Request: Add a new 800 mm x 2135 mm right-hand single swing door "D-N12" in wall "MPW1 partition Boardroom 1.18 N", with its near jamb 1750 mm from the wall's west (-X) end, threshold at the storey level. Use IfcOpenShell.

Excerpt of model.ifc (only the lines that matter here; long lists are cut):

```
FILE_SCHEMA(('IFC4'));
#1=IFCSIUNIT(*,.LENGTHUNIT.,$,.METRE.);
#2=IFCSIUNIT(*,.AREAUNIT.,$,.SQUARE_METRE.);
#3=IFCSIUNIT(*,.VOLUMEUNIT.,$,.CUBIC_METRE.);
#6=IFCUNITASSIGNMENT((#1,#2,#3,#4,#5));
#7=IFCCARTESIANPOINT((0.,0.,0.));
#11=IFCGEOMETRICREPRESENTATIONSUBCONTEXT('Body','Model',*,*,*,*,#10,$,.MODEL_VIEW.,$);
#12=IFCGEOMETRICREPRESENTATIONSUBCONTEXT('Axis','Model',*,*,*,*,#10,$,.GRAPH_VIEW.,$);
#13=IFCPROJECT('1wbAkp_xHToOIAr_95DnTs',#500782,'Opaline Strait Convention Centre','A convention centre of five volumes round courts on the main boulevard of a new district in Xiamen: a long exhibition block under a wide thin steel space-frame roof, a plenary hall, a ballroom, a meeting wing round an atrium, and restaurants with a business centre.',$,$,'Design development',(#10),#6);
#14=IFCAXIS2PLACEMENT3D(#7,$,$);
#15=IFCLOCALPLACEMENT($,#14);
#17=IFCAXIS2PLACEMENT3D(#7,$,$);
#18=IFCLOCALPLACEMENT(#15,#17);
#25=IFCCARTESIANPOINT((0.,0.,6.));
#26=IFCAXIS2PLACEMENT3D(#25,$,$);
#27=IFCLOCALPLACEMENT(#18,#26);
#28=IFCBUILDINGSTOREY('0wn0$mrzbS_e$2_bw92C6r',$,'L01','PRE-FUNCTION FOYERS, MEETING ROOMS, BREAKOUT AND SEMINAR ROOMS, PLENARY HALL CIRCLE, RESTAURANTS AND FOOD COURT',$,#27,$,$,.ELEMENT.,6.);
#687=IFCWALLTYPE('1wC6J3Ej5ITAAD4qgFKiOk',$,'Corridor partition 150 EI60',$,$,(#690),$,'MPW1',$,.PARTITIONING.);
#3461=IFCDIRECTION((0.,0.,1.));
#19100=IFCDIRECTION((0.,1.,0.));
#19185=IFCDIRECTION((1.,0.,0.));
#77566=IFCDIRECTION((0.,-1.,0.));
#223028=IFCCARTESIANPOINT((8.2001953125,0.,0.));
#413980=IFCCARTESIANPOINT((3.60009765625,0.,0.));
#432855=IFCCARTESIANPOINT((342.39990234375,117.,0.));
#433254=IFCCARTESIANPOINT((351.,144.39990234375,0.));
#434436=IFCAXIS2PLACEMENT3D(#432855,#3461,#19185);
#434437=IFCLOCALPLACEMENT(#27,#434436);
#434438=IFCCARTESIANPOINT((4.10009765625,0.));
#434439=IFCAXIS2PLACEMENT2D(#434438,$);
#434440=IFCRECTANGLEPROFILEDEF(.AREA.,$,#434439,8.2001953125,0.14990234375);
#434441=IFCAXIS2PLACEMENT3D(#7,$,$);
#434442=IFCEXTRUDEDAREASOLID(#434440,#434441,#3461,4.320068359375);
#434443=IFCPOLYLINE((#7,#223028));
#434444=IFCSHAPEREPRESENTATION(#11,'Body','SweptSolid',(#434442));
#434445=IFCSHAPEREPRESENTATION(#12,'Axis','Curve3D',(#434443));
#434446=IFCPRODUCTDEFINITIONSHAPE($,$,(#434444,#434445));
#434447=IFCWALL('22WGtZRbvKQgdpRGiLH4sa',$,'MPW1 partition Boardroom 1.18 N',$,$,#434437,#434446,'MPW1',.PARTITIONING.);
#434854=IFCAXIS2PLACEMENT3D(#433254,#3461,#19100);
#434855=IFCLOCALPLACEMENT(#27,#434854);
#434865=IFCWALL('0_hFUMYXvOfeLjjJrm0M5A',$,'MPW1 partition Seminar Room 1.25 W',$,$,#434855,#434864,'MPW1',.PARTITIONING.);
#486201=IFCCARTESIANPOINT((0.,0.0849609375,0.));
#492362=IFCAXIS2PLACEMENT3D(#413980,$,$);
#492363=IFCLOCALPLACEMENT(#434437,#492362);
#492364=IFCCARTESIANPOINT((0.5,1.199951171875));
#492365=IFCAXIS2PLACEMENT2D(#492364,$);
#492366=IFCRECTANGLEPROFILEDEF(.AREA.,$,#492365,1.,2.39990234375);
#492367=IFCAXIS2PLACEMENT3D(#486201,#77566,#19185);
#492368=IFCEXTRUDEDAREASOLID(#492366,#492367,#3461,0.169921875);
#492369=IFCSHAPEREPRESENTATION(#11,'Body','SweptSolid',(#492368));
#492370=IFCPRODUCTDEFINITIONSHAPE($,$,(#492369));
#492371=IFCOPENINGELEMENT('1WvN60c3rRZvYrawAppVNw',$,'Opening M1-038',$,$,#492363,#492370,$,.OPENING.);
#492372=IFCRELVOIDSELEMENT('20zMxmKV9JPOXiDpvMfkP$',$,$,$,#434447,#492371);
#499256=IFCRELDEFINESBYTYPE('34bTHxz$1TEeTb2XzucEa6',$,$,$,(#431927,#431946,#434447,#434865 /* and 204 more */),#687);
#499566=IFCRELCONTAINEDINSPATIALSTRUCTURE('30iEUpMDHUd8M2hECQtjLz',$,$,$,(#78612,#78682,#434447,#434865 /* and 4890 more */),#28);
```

```python
import numpy as np
import ifcopenshell
import ifcopenshell.api.feature
import ifcopenshell.api.geometry
import ifcopenshell.api.root
import ifcopenshell.api.spatial
import ifcopenshell.geom
import ifcopenshell.util.element
import ifcopenshell.util.placement
import ifcopenshell.util.representation
import ifcopenshell.util.shape
import ifcopenshell.util.unit

model = ifcopenshell.open("model.ifc")
unit_scale = ifcopenshell.util.unit.calculate_unit_scale(model)
settings = ifcopenshell.geom.settings()


def volume(element):
    """Net volume in cubic metres, openings subtracted."""
    shape = ifcopenshell.geom.create_shape(settings, element)
    return ifcopenshell.util.shape.get_volume(shape.geometry)


wall = model.by_guid("22WGtZRbvKQgdpRGiLH4sa")
storey = ifcopenshell.util.element.get_container(wall, ifc_class="IfcBuildingStorey")
context = ifcopenshell.util.representation.get_context(model, "Model", "Body", "MODEL_VIEW")
before = volume(wall)

width, height, from_end, sill = 0.8, 2.135, 1.75, 0.0  # metres

# The wall runs along its own X axis, and the end named is its -X end.
wall_shape = ifcopenshell.geom.create_shape(settings, wall)
x, y, z = ifcopenshell.util.shape.get_vertices(wall_shape.geometry).T
start = x.min() + from_end
face, thickness = float(y.min()), float(y.max() - y.min())
wall_matrix = ifcopenshell.util.placement.get_local_placement(wall.ObjectPlacement)
level = ifcopenshell.util.placement.get_local_placement(storey.ObjectPlacement)[2, 3]


def in_wall(x, y):
    """Placement at x, y metres in the wall's axes, at sill height."""
    matrix = wall_matrix.copy()
    matrix[:, 3] = wall_matrix @ np.array([x / unit_scale, y / unit_scale, 0.0, 1.0])
    matrix[2, 3] = level + sill / unit_scale
    return matrix


# Opening: a box that overshoots both wall faces by 50 mm.
opening = ifcopenshell.api.root.create_entity(model, ifc_class="IfcOpeningElement", predefined_type="OPENING")
box = ifcopenshell.api.geometry.add_wall_representation(
    model, context=context, length=width, height=height, thickness=thickness + 0.1
)
ifcopenshell.api.geometry.assign_representation(model, product=opening, representation=box)
ifcopenshell.api.geometry.edit_object_placement(model, product=opening, matrix=in_wall(start, face - 0.05), is_si=False)
ifcopenshell.api.feature.add_feature(model, feature=opening, element=wall)

door = ifcopenshell.api.root.create_entity(model, ifc_class="IfcDoor", name="D-N12", predefined_type="DOOR")
door.OverallWidth, door.OverallHeight = width / unit_scale, height / unit_scale
door.OperationType = "SINGLE_SWING_RIGHT"
body = ifcopenshell.api.geometry.add_door_representation(
    model,
    context=context,
    overall_width=door.OverallWidth,
    overall_height=door.OverallHeight,
    operation_type="SINGLE_SWING_RIGHT",
    lining_properties={"LiningDepth": thickness / unit_scale, "ThresholdDepth": thickness / unit_scale},
)
ifcopenshell.api.geometry.assign_representation(model, product=door, representation=body)
ifcopenshell.api.spatial.assign_container(model, products=[door], relating_structure=storey)
ifcopenshell.api.feature.add_filling(model, opening=opening, element=door)

# The lining spans the wall, so the door starts at the wall face.
ifcopenshell.api.geometry.edit_object_placement(model, product=door, matrix=in_wall(start, face), is_si=False)

after = volume(wall)

print(f"wall volume {before:.3f} -> {after:.3f} m3")

model.write("model_rev.ifc")
```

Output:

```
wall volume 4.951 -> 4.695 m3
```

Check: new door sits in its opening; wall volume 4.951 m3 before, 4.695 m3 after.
